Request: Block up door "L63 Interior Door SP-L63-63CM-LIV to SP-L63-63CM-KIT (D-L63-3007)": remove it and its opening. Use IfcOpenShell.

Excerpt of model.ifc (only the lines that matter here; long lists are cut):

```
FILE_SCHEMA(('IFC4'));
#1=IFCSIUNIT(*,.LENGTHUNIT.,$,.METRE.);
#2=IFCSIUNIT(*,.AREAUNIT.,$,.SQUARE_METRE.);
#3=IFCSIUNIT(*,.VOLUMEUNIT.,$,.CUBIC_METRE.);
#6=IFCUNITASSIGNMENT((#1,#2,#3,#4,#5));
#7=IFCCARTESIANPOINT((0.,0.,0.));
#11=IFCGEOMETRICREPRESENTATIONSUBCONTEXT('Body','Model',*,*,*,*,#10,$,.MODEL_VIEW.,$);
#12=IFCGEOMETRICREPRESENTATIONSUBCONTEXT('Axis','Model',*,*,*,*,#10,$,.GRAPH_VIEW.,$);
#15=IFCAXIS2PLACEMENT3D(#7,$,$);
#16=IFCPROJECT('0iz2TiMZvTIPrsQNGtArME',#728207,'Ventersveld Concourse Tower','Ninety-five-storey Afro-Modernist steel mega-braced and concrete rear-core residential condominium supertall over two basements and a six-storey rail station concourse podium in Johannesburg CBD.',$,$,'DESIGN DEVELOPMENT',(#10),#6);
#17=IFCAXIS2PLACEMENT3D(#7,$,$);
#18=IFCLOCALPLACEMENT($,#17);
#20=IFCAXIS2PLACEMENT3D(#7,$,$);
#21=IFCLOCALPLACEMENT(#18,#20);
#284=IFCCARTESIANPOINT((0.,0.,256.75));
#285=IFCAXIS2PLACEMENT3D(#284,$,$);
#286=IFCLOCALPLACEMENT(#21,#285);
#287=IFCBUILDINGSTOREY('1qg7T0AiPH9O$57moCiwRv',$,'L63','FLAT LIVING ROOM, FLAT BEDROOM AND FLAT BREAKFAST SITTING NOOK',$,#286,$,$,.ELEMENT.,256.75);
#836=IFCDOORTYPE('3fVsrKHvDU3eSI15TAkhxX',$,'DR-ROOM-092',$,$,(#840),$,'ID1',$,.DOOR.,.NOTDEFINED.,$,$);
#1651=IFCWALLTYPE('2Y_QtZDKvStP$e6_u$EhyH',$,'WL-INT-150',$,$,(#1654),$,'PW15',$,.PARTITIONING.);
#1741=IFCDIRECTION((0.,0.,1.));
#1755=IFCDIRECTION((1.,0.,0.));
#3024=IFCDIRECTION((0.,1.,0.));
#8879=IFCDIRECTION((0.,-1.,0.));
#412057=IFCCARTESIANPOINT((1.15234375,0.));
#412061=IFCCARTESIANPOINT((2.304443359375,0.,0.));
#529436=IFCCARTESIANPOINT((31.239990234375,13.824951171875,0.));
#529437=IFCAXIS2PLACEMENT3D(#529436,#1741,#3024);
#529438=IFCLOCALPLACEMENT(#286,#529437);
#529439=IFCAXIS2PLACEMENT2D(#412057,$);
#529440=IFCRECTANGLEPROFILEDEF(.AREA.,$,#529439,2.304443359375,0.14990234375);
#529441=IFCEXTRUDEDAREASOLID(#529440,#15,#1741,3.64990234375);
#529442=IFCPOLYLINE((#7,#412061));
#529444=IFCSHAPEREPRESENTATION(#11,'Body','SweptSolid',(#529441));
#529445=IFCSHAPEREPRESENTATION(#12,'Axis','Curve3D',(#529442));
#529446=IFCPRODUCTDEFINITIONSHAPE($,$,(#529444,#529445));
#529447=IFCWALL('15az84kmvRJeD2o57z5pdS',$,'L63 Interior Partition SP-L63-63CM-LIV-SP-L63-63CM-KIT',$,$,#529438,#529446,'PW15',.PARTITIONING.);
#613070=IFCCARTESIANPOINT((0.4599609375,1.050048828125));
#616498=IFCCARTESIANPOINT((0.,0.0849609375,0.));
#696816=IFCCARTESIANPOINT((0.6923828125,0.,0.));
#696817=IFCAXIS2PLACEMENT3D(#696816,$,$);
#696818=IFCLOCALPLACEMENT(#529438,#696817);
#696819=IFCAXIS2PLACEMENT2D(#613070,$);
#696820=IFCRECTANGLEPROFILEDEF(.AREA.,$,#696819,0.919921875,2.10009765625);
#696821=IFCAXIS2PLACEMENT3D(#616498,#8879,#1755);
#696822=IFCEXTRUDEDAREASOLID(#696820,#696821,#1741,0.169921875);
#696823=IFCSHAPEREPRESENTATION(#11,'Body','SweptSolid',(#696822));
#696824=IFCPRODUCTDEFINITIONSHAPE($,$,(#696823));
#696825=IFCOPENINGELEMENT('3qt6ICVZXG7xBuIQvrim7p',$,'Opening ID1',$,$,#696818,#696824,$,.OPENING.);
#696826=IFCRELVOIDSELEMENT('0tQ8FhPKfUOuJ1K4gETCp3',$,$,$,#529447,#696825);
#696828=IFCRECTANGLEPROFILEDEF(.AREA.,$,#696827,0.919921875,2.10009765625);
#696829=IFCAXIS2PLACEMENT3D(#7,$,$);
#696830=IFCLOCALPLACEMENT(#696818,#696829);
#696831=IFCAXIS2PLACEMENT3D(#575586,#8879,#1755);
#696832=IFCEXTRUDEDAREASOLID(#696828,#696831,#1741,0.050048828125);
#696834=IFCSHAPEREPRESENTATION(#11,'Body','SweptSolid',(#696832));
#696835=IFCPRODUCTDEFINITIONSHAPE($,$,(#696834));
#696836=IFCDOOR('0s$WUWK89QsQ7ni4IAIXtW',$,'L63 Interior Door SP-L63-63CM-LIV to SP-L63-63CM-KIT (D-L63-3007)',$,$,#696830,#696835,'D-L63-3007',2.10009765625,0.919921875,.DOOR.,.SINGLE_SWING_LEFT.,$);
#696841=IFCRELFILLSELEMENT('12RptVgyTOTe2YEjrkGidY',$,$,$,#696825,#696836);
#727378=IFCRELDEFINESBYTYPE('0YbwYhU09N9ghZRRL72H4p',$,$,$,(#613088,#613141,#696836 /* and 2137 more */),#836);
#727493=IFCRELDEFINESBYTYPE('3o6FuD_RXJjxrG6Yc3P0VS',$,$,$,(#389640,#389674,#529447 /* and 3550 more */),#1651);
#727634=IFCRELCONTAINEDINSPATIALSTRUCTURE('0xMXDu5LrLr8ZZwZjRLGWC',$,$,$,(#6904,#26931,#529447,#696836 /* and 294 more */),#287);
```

```python
import ifcopenshell
import ifcopenshell.api.feature
import ifcopenshell.api.root
import ifcopenshell.geom
import ifcopenshell.util.shape

model = ifcopenshell.open("model.ifc")
settings = ifcopenshell.geom.settings()


def volume(element):
    """Net volume in cubic metres, openings subtracted."""
    shape = ifcopenshell.geom.create_shape(settings, element)
    return ifcopenshell.util.shape.get_volume(shape.geometry)


door = model.by_guid("0s$WUWK89QsQ7ni4IAIXtW")
opening = door.FillsVoids[0].RelatingOpeningElement
wall = opening.VoidsElements[0].RelatingBuildingElement
before = volume(wall)

ifcopenshell.api.root.remove_product(model, product=door)
ifcopenshell.api.feature.remove_feature(model, feature=opening)

after = volume(wall)

print(f"wall volume {before:.3f} -> {after:.3f} m3")

model.write("model_edited.ifc")
```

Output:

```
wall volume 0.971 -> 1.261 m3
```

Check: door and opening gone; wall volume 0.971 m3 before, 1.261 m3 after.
